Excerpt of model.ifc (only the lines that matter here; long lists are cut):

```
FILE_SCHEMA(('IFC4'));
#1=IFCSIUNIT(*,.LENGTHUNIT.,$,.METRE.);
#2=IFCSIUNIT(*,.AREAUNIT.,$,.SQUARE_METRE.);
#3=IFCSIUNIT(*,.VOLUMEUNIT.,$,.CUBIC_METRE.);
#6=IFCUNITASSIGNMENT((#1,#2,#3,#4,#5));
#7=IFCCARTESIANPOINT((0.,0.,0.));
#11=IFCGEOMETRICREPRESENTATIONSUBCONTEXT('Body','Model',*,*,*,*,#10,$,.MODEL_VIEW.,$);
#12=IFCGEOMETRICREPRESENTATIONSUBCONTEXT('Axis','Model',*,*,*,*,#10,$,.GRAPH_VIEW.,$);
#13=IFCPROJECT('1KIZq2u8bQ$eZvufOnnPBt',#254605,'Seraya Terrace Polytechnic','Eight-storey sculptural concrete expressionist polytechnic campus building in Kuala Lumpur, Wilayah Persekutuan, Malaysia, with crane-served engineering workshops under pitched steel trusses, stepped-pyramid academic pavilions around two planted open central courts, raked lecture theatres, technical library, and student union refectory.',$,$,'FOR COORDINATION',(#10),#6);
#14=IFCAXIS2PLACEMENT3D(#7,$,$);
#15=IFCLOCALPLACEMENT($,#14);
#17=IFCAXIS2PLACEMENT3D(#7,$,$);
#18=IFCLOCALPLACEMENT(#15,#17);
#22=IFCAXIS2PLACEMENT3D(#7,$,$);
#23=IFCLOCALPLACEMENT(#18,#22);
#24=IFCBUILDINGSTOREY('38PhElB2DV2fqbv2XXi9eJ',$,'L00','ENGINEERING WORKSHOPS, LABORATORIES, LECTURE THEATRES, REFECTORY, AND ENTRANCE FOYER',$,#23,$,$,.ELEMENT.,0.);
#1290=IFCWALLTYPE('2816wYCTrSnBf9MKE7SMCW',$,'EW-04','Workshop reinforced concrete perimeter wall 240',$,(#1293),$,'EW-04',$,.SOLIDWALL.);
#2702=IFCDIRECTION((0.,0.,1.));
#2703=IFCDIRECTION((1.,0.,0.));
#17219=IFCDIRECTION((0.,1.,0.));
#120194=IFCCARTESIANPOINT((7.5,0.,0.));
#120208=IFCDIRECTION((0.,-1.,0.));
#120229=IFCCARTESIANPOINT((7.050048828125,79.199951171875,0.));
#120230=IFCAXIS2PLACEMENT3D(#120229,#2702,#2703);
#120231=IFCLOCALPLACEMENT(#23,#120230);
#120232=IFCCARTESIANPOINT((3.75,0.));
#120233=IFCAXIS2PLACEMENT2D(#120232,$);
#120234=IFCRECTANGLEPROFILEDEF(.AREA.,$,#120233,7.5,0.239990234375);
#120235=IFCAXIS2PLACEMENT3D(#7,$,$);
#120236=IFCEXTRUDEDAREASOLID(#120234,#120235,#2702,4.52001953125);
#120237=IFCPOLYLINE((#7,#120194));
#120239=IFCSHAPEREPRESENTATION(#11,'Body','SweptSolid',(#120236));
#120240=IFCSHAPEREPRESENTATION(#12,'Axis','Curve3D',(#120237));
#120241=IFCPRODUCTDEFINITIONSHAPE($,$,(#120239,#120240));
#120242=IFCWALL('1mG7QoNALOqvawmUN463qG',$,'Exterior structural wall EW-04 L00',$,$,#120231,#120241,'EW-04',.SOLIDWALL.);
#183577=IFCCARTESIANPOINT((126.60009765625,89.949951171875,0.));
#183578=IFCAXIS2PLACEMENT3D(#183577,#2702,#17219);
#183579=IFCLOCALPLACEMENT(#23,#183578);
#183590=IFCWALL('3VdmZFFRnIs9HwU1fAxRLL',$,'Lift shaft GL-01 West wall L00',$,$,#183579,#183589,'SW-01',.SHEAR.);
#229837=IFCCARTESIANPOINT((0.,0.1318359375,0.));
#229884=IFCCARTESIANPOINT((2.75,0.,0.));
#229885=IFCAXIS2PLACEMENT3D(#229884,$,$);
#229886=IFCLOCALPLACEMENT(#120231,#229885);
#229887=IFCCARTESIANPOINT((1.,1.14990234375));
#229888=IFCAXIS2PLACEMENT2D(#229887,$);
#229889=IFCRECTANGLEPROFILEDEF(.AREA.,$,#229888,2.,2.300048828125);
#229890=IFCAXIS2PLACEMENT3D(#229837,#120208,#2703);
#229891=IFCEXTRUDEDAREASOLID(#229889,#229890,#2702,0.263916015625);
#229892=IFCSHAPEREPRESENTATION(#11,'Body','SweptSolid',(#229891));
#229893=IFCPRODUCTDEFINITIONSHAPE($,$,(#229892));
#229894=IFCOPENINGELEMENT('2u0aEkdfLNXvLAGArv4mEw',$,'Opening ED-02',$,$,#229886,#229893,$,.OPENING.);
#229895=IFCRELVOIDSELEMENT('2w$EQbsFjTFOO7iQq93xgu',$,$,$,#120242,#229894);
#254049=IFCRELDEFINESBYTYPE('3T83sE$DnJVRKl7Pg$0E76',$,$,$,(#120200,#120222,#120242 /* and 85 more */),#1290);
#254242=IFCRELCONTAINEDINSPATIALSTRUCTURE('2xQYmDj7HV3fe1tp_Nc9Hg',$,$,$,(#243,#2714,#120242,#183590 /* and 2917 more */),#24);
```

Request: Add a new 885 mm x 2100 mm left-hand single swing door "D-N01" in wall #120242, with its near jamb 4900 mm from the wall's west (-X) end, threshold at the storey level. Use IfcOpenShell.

```python
import numpy as np
import ifcopenshell
import ifcopenshell.api.feature
import ifcopenshell.api.geometry
import ifcopenshell.api.root
import ifcopenshell.api.spatial
import ifcopenshell.geom
import ifcopenshell.util.element
import ifcopenshell.util.placement
import ifcopenshell.util.representation
import ifcopenshell.util.shape
import ifcopenshell.util.unit

model = ifcopenshell.open("model.ifc")
unit_scale = ifcopenshell.util.unit.calculate_unit_scale(model)
settings = ifcopenshell.geom.settings()


def volume(element):
    """Net volume in cubic metres, openings subtracted."""
    shape = ifcopenshell.geom.create_shape(settings, element)
    return ifcopenshell.util.shape.get_volume(shape.geometry)


wall = model.by_guid("1mG7QoNALOqvawmUN463qG")
storey = ifcopenshell.util.element.get_container(wall, ifc_class="IfcBuildingStorey")
context = ifcopenshell.util.representation.get_context(model, "Model", "Body", "MODEL_VIEW")
before = volume(wall)

width, height, from_end, sill = 0.885, 2.1, 4.9, 0.0  # metres

# The wall runs along its own X axis, and the end named is its -X end.
wall_shape = ifcopenshell.geom.create_shape(settings, wall)
x, y, z = ifcopenshell.util.shape.get_vertices(wall_shape.geometry).T
start = x.min() + from_end
face, thickness = float(y.min()), float(y.max() - y.min())
wall_matrix = ifcopenshell.util.placement.get_local_placement(wall.ObjectPlacement)
level = ifcopenshell.util.placement.get_local_placement(storey.ObjectPlacement)[2, 3]


def in_wall(x, y):
    """Placement at x, y metres in the wall's axes, at sill height."""
    matrix = wall_matrix.copy()
    matrix[:, 3] = wall_matrix @ np.array([x / unit_scale, y / unit_scale, 0.0, 1.0])
    matrix[2, 3] = level + sill / unit_scale
    return matrix


# Opening: a box that overshoots both wall faces by 50 mm.
opening = ifcopenshell.api.root.create_entity(model, ifc_class="IfcOpeningElement", predefined_type="OPENING")
box = ifcopenshell.api.geometry.add_wall_representation(
    model, context=context, length=width, height=height, thickness=thickness + 0.1
)
ifcopenshell.api.geometry.assign_representation(model, product=opening, representation=box)
ifcopenshell.api.geometry.edit_object_placement(model, product=opening, matrix=in_wall(start, face - 0.05), is_si=False)
ifcopenshell.api.feature.add_feature(model, feature=opening, element=wall)

door = ifcopenshell.api.root.create_entity(model, ifc_class="IfcDoor", name="D-N01", predefined_type="DOOR")
door.OverallWidth, door.OverallHeight = width / unit_scale, height / unit_scale
door.OperationType = "SINGLE_SWING_LEFT"
body = ifcopenshell.api.geometry.add_door_representation(
    model,
    context=context,
    overall_width=door.OverallWidth,
    overall_height=door.OverallHeight,
    operation_type="SINGLE_SWING_LEFT",
    lining_properties={"LiningDepth": thickness / unit_scale, "ThresholdDepth": thickness / unit_scale},
)
ifcopenshell.api.geometry.assign_representation(model, product=door, representation=body)
ifcopenshell.api.spatial.assign_container(model, products=[door], relating_structure=storey)
ifcopenshell.api.feature.add_filling(model, opening=opening, element=door)

# The lining spans the wall, so the door starts at the wall face.
ifcopenshell.api.geometry.edit_object_placement(model, product=door, matrix=in_wall(start, face), is_si=False)

after = volume(wall)

print(f"wall volume {before:.3f} -> {after:.3f} m3")

model.write("model_edited.ifc")
```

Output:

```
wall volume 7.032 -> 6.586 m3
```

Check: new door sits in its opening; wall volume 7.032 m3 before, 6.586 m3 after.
